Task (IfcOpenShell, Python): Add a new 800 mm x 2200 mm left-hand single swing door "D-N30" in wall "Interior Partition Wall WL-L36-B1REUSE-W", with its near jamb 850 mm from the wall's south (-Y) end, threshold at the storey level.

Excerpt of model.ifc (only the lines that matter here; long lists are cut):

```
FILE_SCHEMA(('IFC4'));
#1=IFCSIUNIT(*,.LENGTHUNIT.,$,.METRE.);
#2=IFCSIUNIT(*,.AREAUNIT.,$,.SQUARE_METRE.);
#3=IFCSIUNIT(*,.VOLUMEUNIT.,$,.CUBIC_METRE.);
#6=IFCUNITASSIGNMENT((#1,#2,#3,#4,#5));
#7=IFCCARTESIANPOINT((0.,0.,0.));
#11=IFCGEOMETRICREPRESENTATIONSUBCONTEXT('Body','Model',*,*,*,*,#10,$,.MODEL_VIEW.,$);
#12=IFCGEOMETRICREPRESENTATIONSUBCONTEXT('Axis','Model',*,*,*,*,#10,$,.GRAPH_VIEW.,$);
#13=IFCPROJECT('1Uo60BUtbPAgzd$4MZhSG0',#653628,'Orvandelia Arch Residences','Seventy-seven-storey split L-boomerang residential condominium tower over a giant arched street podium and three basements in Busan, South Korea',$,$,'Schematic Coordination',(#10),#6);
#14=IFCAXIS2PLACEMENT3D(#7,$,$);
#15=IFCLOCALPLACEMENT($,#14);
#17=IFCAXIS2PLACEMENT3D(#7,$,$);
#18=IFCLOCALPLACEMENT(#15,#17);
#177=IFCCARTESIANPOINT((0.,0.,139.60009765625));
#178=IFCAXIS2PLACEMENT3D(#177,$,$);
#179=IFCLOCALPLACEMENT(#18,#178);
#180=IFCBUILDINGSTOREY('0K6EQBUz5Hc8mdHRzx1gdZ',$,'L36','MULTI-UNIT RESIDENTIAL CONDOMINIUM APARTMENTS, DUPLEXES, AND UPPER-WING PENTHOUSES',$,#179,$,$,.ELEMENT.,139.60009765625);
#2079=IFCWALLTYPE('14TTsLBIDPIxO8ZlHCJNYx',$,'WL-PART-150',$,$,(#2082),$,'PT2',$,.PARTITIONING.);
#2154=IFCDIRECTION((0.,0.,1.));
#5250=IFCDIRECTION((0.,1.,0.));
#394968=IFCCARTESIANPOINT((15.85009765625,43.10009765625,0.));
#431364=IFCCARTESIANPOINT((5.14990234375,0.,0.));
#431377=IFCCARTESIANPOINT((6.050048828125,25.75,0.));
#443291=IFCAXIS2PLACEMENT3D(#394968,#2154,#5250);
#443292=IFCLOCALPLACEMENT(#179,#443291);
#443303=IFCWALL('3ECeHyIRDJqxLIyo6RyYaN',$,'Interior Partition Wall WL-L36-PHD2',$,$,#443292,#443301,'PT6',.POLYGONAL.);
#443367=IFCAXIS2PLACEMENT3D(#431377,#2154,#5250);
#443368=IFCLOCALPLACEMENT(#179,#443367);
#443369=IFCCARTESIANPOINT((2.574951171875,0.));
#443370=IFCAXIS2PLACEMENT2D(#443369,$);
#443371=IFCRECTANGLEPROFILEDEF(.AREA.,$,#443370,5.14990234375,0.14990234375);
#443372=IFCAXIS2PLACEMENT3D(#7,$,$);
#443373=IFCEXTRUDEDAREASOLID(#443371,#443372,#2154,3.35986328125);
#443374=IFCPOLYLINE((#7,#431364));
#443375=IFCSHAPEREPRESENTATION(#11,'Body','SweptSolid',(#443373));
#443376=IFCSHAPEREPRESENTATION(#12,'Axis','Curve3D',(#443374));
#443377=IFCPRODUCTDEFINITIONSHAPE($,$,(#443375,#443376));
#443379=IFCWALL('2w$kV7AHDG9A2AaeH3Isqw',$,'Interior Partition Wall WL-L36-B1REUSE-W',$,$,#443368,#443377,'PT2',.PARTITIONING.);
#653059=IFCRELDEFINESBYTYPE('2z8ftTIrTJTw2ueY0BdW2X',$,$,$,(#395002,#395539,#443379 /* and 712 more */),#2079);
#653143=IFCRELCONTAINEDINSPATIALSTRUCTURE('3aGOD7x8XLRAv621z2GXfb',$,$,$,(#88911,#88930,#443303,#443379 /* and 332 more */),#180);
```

```python
import numpy as np
import ifcopenshell
import ifcopenshell.api.feature
import ifcopenshell.api.geometry
import ifcopenshell.api.root
import ifcopenshell.api.spatial
import ifcopenshell.geom
import ifcopenshell.util.element
import ifcopenshell.util.placement
import ifcopenshell.util.representation
import ifcopenshell.util.shape
import ifcopenshell.util.unit

model = ifcopenshell.open("model.ifc")
unit_scale = ifcopenshell.util.unit.calculate_unit_scale(model)
settings = ifcopenshell.geom.settings()


def volume(element):
    """Net volume in cubic metres, openings subtracted."""
    shape = ifcopenshell.geom.create_shape(settings, element)
    return ifcopenshell.util.shape.get_volume(shape.geometry)


wall = model.by_guid("2w$kV7AHDG9A2AaeH3Isqw")
storey = ifcopenshell.util.element.get_container(wall, ifc_class="IfcBuildingStorey")
context = ifcopenshell.util.representation.get_context(model, "Model", "Body", "MODEL_VIEW")
before = volume(wall)

width, height, from_end, sill = 0.8, 2.2, 0.85, 0.0  # metres

# The wall runs along its own X axis, and the end named is its -X end.
wall_shape = ifcopenshell.geom.create_shape(settings, wall)
x, y, z = ifcopenshell.util.shape.get_vertices(wall_shape.geometry).T
start = x.min() + from_end
face, thickness = float(y.min()), float(y.max() - y.min())
wall_matrix = ifcopenshell.util.placement.get_local_placement(wall.ObjectPlacement)
level = ifcopenshell.util.placement.get_local_placement(storey.ObjectPlacement)[2, 3]


def in_wall(x, y):
    """Placement at x, y metres in the wall's axes, at sill height."""
    matrix = wall_matrix.copy()
    matrix[:, 3] = wall_matrix @ np.array([x / unit_scale, y / unit_scale, 0.0, 1.0])
    matrix[2, 3] = level + sill / unit_scale
    return matrix


# Opening: a box that overshoots both wall faces by 50 mm.
opening = ifcopenshell.api.root.create_entity(model, ifc_class="IfcOpeningElement", predefined_type="OPENING")
box = ifcopenshell.api.geometry.add_wall_representation(
    model, context=context, length=width, height=height, thickness=thickness + 0.1
)
ifcopenshell.api.geometry.assign_representation(model, product=opening, representation=box)
ifcopenshell.api.geometry.edit_object_placement(model, product=opening, matrix=in_wall(start, face - 0.05), is_si=False)
ifcopenshell.api.feature.add_feature(model, feature=opening, element=wall)

door = ifcopenshell.api.root.create_entity(model, ifc_class="IfcDoor", name="D-N30", predefined_type="DOOR")
door.OverallWidth, door.OverallHeight = width / unit_scale, height / unit_scale
door.OperationType = "SINGLE_SWING_LEFT"
body = ifcopenshell.api.geometry.add_door_representation(
    model,
    context=context,
    overall_width=door.OverallWidth,
    overall_height=door.OverallHeight,
    operation_type="SINGLE_SWING_LEFT",
    lining_properties={"LiningDepth": thickness / unit_scale, "ThresholdDepth": thickness / unit_scale},
)
ifcopenshell.api.geometry.assign_representation(model, product=door, representation=body)
ifcopenshell.api.spatial.assign_container(model, products=[door], relating_structure=storey)
ifcopenshell.api.feature.add_filling(model, opening=opening, element=door)

# The lining spans the wall, so the door starts at the wall face.
ifcopenshell.api.geometry.edit_object_placement(model, product=door, matrix=in_wall(start, face), is_si=False)

after = volume(wall)

print(f"wall volume {before:.3f} -> {after:.3f} m3")

model.write("model-out.ifc")
```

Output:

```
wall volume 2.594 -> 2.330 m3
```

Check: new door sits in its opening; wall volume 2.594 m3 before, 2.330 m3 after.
